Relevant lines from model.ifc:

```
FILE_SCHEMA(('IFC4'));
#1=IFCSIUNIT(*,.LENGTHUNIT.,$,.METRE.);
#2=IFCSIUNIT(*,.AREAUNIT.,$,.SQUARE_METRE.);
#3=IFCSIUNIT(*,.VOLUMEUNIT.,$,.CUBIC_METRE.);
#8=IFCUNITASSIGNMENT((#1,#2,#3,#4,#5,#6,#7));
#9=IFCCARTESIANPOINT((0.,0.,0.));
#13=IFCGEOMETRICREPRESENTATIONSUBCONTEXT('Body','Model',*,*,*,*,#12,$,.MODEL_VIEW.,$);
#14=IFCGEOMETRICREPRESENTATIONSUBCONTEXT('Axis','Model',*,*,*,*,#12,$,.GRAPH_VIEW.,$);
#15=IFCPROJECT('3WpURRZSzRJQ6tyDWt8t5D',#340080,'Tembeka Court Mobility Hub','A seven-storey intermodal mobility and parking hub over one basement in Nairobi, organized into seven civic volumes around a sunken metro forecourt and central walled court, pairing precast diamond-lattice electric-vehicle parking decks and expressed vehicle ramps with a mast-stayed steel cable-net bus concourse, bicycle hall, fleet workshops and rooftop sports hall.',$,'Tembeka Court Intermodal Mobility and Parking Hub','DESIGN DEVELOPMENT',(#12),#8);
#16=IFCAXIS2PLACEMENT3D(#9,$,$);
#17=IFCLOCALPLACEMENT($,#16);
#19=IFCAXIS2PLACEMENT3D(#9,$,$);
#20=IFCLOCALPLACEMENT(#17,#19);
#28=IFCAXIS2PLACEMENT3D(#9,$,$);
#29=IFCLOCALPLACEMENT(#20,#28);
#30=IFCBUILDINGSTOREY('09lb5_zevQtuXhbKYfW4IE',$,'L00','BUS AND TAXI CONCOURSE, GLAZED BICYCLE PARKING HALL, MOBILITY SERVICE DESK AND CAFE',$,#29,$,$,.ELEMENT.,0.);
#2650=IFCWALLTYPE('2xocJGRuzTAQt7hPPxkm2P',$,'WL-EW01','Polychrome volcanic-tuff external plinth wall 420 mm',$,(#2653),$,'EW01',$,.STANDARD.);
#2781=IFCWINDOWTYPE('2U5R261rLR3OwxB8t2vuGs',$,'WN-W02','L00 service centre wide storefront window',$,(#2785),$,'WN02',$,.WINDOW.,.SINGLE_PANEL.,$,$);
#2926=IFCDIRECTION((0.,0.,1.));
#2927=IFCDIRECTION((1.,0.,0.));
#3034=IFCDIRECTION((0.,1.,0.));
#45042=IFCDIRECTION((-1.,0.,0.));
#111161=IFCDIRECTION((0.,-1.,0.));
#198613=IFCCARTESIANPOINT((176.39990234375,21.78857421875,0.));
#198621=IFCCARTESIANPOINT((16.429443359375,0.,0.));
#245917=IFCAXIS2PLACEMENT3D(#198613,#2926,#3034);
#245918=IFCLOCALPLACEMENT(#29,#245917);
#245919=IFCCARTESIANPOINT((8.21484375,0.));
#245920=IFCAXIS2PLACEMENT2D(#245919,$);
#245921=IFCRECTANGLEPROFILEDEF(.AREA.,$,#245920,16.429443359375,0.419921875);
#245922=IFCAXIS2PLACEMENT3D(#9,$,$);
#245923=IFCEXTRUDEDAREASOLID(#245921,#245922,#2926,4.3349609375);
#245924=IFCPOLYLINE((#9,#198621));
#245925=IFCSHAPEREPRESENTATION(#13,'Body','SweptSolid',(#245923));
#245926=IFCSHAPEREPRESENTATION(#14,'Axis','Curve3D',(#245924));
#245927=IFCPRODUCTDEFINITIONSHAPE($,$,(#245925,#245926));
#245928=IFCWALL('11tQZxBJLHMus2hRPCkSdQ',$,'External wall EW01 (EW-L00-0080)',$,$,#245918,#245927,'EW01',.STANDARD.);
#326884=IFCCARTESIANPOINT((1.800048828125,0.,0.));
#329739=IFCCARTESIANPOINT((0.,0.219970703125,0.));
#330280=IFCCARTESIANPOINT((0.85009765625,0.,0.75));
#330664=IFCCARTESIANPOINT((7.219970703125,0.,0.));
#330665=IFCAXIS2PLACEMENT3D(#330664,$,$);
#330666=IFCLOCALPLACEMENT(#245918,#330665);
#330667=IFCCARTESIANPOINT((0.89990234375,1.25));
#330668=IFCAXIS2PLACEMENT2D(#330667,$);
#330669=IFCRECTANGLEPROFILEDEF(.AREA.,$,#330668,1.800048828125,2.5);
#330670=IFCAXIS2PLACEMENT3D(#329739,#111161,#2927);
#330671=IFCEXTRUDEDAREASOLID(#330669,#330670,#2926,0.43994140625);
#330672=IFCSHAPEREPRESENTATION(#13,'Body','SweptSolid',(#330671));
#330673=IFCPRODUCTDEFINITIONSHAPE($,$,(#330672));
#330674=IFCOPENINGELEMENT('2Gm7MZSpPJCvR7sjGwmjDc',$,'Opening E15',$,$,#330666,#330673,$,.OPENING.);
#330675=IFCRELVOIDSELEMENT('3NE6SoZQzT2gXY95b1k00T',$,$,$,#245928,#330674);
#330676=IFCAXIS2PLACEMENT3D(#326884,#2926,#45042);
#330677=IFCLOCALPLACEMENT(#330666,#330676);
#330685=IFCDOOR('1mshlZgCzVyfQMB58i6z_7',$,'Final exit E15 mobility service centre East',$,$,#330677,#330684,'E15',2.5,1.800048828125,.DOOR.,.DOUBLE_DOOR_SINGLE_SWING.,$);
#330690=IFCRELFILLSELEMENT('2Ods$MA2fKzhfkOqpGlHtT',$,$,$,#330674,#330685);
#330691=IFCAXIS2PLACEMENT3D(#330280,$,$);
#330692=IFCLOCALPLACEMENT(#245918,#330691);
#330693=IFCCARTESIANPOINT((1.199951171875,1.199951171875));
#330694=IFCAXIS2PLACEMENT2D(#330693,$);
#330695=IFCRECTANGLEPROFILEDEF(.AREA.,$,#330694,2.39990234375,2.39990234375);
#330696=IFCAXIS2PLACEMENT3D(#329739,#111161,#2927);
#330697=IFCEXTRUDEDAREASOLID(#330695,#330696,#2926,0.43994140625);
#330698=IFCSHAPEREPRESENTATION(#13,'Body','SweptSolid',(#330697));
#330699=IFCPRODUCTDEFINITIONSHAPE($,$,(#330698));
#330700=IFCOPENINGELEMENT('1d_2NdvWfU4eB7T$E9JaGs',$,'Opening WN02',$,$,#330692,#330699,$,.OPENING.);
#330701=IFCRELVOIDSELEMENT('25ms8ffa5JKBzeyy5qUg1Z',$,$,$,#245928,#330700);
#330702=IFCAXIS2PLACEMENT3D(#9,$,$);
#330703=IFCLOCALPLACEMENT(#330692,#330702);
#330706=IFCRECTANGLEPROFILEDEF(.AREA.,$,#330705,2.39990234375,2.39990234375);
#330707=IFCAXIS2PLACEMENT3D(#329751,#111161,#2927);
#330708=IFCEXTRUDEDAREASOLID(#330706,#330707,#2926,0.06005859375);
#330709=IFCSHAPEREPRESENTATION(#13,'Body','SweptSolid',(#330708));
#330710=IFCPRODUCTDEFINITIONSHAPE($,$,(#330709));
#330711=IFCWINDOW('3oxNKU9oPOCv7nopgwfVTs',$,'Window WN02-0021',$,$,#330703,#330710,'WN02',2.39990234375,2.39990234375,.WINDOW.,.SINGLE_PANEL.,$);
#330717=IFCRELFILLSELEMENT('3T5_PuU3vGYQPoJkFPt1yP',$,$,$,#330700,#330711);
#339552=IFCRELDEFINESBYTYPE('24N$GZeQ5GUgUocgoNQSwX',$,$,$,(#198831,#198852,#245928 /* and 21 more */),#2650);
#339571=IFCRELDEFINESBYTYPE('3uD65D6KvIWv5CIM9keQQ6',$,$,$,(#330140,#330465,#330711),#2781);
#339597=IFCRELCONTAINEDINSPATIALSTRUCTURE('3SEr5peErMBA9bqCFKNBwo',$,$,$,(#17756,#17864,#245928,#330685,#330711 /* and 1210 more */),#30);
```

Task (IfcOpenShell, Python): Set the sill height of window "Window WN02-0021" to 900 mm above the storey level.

```python
import numpy as np
import ifcopenshell
import ifcopenshell.api.geometry
import ifcopenshell.geom
import ifcopenshell.util.element
import ifcopenshell.util.placement
import ifcopenshell.util.shape
import ifcopenshell.util.unit

model = ifcopenshell.open("model.ifc")
unit_scale = ifcopenshell.util.unit.calculate_unit_scale(model)

window = model.by_id(330711)
opening = window.FillsVoids[0].RelatingOpeningElement
storey = ifcopenshell.util.element.get_container(window, ifc_class="IfcBuildingStorey")
level = ifcopenshell.util.placement.get_local_placement(storey.ObjectPlacement)[2, 3]

# The opening's origin need not be at the sill, so measure its lowest point.
shape = ifcopenshell.geom.create_shape(ifcopenshell.geom.settings(), opening)
bottom = ifcopenshell.util.shape.get_shape_bottom_elevation(shape, shape.geometry) / unit_scale
dz = level + 0.9 / unit_scale - bottom

shift = np.array([0.0, 0.0, dz])
# The window is placed relative to its opening, so it follows when the opening moves.
matrix = ifcopenshell.util.placement.get_local_placement(opening.ObjectPlacement)
matrix[:3, 3] += shift
ifcopenshell.api.geometry.edit_object_placement(
    model, product=opening, matrix=matrix, is_si=False, should_transform_children=True
)

print(f"moved by {dz * unit_scale:+.3f} m")

model.write("model-out.ifc")
```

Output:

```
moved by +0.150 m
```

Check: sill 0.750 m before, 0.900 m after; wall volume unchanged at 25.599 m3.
